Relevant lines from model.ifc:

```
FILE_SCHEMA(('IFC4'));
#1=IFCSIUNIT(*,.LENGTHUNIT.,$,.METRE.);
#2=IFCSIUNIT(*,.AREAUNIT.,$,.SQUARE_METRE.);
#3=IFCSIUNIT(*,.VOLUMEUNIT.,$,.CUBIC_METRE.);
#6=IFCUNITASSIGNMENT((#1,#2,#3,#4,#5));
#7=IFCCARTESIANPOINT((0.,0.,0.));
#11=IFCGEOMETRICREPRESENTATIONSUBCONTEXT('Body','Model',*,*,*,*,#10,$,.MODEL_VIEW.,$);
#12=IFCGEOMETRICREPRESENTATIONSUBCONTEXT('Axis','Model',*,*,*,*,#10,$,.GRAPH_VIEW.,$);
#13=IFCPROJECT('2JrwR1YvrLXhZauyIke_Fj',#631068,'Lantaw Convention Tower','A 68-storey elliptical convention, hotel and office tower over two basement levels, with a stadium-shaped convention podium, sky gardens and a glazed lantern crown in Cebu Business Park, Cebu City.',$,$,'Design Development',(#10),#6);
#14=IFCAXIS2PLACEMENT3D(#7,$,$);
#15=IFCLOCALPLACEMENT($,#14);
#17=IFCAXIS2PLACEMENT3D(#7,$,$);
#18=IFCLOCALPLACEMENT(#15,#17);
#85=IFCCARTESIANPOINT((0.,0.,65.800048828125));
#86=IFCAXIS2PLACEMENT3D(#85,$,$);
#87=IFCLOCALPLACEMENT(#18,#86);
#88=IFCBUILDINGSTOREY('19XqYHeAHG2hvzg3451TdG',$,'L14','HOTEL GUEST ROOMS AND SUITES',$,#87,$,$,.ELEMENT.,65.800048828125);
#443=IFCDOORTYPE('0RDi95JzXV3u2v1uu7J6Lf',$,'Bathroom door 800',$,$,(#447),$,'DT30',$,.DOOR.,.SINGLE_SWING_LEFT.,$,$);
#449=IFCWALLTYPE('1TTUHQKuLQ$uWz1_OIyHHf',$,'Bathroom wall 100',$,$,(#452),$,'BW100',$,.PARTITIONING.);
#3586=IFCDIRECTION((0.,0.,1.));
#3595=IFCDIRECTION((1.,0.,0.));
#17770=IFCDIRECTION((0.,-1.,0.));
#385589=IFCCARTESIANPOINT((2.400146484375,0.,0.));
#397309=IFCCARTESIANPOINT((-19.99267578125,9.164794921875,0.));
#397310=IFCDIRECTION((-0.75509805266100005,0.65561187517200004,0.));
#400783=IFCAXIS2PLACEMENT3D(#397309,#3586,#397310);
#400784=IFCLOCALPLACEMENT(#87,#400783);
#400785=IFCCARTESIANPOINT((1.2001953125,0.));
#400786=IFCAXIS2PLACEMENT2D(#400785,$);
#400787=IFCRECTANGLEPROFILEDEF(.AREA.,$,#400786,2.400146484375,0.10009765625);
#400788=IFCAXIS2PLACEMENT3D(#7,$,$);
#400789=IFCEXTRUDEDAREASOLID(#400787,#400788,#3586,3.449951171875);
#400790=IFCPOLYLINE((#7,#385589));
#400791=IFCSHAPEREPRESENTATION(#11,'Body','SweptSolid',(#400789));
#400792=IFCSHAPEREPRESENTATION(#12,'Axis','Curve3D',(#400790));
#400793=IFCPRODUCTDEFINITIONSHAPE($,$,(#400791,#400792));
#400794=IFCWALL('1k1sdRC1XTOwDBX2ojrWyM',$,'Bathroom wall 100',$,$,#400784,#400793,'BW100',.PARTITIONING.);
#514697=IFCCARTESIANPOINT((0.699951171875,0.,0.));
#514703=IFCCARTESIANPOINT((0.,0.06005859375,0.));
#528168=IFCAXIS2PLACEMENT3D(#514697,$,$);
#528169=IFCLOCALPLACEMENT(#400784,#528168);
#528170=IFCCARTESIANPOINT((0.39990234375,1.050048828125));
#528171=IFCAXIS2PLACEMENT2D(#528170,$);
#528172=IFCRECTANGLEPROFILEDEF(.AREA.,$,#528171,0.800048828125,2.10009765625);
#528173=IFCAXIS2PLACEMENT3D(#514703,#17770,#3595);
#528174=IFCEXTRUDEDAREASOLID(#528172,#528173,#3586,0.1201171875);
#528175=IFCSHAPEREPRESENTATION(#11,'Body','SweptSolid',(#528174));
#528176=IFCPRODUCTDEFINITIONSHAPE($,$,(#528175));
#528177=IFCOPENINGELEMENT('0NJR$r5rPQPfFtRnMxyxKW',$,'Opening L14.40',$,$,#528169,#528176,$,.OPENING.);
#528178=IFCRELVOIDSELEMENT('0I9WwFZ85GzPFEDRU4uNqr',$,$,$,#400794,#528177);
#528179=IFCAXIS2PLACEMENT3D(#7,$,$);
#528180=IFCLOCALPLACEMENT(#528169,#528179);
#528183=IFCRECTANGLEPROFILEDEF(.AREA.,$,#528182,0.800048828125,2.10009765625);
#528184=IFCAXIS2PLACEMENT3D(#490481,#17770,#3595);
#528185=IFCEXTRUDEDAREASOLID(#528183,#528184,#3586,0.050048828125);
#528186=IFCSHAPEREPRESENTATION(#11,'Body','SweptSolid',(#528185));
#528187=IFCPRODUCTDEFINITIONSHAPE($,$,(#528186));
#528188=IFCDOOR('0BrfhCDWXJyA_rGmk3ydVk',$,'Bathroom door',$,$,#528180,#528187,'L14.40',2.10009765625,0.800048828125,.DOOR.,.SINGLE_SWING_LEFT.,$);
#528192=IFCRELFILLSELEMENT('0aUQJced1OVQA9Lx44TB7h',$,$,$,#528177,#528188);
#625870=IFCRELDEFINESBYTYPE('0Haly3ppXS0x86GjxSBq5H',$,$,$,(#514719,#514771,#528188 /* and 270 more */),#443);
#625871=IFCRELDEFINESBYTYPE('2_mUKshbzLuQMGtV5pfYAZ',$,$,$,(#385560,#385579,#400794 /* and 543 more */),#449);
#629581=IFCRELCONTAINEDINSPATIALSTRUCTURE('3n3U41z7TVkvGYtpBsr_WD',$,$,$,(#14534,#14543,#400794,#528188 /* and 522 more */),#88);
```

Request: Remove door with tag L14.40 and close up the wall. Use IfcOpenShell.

```python
import ifcopenshell
import ifcopenshell.api.feature
import ifcopenshell.api.root
import ifcopenshell.geom
import ifcopenshell.util.shape

model = ifcopenshell.open("model.ifc")
settings = ifcopenshell.geom.settings()


def volume(element):
    """Net volume in cubic metres, openings subtracted."""
    shape = ifcopenshell.geom.create_shape(settings, element)
    return ifcopenshell.util.shape.get_volume(shape.geometry)


door = model.by_guid("0BrfhCDWXJyA_rGmk3ydVk")
opening = door.FillsVoids[0].RelatingOpeningElement
wall = opening.VoidsElements[0].RelatingBuildingElement
before = volume(wall)

ifcopenshell.api.root.remove_product(model, product=door)
ifcopenshell.api.feature.remove_feature(model, feature=opening)

after = volume(wall)

print(f"wall volume {before:.3f} -> {after:.3f} m3")

model.write("model_edited.ifc")
```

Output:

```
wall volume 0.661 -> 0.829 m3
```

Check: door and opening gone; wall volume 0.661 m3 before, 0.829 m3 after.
